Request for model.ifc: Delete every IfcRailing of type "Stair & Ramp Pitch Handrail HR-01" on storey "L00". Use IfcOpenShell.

First a look at what the model holds.

```python
import ifcopenshell
import ifcopenshell.util.element

model = ifcopenshell.open("model.ifc")
print(model.schema)
storey = next(s for s in model.by_type("IfcBuildingStorey") if s.Name == "L00")
railings = [e for e in ifcopenshell.util.element.get_decomposition(storey) if e.is_a("IfcRailing")]
seen = {}
for e in railings:
    element_type = ifcopenshell.util.element.get_type(e)
    name = element_type.Name if element_type not in (None, e) else None
    seen[name] = seen.get(name, 0) + 1
for name, count in sorted(seen.items(), key=str):
    print(count, "x", name)
```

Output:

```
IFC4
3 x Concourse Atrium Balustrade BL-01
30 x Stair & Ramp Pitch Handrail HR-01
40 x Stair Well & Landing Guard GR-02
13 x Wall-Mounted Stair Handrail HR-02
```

```python
import ifcopenshell
import ifcopenshell.api.root
import ifcopenshell.util.element

model = ifcopenshell.open("model.ifc")

storey = next(s for s in model.by_type("IfcBuildingStorey") if s.Name == "L00")
railings = [e for e in ifcopenshell.util.element.get_decomposition(storey) if e.is_a("IfcRailing")]
targets = [e for e in railings if (t := ifcopenshell.util.element.get_type(e)) not in (None, e) and t.Name == "Stair & Ramp Pitch Handrail HR-01"]

for e in targets:
    ifcopenshell.api.root.remove_product(model, product=e)
print(len(targets), "removed")

model.write("model_rev.ifc")
```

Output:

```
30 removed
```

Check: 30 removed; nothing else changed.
